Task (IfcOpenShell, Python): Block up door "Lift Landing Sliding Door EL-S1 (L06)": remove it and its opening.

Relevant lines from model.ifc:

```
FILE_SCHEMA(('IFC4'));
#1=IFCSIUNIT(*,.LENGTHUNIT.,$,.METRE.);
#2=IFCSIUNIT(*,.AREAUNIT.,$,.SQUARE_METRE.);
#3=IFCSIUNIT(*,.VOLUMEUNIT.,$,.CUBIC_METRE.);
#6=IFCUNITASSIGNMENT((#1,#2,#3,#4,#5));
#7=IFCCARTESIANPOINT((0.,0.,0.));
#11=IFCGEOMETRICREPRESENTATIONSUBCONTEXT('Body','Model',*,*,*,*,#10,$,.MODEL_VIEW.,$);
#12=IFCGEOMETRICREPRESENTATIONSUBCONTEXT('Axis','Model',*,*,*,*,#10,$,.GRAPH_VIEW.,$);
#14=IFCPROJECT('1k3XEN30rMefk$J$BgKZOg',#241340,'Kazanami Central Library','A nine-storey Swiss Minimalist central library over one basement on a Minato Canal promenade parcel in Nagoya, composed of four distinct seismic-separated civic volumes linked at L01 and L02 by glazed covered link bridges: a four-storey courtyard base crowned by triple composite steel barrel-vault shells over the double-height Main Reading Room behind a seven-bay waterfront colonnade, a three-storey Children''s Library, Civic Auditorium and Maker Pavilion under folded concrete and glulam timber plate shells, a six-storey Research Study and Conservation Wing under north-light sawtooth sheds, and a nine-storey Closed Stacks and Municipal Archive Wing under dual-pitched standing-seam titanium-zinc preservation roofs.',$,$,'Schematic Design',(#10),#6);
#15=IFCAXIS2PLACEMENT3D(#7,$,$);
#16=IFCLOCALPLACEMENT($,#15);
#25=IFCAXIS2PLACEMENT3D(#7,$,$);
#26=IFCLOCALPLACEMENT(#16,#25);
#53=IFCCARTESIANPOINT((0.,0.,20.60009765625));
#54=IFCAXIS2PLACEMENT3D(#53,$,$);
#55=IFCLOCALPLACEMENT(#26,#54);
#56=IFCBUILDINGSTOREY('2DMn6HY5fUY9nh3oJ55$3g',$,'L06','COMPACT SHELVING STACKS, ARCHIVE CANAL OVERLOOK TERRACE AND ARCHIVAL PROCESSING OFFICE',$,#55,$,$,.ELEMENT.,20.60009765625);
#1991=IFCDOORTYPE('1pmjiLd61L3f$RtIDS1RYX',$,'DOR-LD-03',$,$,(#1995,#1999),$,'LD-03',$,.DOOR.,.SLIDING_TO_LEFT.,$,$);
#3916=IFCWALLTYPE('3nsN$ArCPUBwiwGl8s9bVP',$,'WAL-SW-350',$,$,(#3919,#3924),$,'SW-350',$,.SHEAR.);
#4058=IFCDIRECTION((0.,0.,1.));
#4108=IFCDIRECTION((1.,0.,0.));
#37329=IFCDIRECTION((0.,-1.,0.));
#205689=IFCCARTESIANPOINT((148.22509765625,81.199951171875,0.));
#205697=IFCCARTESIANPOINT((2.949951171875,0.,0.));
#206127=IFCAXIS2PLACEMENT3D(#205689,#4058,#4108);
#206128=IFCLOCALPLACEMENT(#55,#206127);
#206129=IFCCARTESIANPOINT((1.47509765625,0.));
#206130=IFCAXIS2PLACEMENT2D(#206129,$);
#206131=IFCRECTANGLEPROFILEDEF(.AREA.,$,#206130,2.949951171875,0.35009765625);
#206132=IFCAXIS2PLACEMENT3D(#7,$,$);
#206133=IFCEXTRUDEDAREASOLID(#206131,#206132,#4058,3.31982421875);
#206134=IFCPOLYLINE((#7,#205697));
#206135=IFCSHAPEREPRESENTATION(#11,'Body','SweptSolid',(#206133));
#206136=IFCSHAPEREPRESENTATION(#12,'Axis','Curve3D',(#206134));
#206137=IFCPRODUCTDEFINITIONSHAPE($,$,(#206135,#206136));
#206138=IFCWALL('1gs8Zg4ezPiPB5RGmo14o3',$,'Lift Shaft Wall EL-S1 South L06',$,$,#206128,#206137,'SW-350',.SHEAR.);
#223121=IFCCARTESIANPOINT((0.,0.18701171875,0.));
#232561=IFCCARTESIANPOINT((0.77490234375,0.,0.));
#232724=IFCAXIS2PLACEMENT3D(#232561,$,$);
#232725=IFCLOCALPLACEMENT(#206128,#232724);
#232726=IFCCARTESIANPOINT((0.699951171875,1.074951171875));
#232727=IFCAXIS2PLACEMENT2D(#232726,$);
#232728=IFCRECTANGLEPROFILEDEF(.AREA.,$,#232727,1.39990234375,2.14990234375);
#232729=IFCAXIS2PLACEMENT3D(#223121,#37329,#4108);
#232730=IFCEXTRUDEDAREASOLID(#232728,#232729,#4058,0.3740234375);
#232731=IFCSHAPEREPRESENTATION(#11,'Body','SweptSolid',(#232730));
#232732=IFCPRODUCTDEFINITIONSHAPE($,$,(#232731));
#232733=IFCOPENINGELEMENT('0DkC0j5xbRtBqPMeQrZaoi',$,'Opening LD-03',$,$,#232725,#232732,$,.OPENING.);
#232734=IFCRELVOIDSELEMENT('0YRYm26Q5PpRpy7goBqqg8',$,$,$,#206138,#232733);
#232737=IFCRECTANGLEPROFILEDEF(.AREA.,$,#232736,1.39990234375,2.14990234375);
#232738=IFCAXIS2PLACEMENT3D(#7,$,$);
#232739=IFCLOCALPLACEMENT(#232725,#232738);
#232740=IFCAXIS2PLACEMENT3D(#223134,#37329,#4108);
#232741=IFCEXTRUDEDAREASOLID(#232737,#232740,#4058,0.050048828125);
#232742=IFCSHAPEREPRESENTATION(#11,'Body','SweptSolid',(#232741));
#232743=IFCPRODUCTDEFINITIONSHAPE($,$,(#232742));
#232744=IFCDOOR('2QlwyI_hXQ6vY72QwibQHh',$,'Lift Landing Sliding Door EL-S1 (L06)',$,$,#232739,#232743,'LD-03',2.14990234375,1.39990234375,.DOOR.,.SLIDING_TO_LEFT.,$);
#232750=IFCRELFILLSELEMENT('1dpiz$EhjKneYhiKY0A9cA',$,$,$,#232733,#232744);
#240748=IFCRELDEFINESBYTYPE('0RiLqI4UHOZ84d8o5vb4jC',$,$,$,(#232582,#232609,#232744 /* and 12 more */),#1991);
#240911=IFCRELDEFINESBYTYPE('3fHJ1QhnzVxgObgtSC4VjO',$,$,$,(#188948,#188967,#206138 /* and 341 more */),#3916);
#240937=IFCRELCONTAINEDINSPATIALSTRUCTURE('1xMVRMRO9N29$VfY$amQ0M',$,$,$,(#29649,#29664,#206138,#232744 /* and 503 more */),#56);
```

```python
import ifcopenshell
import ifcopenshell.api.feature
import ifcopenshell.api.root
import ifcopenshell.geom
import ifcopenshell.util.shape

model = ifcopenshell.open("model.ifc")
settings = ifcopenshell.geom.settings()


def volume(element):
    """Net volume in cubic metres, openings subtracted."""
    shape = ifcopenshell.geom.create_shape(settings, element)
    return ifcopenshell.util.shape.get_volume(shape.geometry)


door = model.by_id(232744)
opening = door.FillsVoids[0].RelatingOpeningElement
wall = opening.VoidsElements[0].RelatingBuildingElement
before = volume(wall)

ifcopenshell.api.root.remove_product(model, product=door)
ifcopenshell.api.feature.remove_feature(model, feature=opening)

after = volume(wall)

print(f"wall volume {before:.3f} -> {after:.3f} m3")

model.write("model-out.ifc")
```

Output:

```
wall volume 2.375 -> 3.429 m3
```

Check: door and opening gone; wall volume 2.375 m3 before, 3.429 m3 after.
